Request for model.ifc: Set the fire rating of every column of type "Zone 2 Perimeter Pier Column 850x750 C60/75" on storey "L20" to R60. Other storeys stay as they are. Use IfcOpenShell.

First a look at what the model holds.

```python
import ifcopenshell
import ifcopenshell.util.element

model = ifcopenshell.open("model.ifc")
print(model.schema)
storey = next(s for s in model.by_type("IfcBuildingStorey") if s.Name == "L20")
columns = [e for e in ifcopenshell.util.element.get_decomposition(storey) if e.is_a("IfcColumn")]
seen = {}
for e in columns:
    element_type = ifcopenshell.util.element.get_type(e)
    key = (element_type.Name if element_type != e and element_type else None, ifcopenshell.util.element.get_pset(e, "Pset_ColumnCommon", "FireRating"))
    seen[key] = seen.get(key, 0) + 1
for (name, value), count in sorted(seen.items(), key=str):
    print(count, "x", name, "|", value)
```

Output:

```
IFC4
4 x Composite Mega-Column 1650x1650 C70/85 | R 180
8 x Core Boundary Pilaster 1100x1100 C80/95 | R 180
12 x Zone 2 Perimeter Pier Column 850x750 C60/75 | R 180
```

```python
import ifcopenshell
import ifcopenshell.api.pset
import ifcopenshell.util.element

model = ifcopenshell.open("model.ifc")

storey = next(s for s in model.by_type("IfcBuildingStorey") if s.Name == "L20")
columns = [e for e in ifcopenshell.util.element.get_decomposition(storey) if e.is_a("IfcColumn")]

count = 0
for e in columns:
    element_type = ifcopenshell.util.element.get_type(e)
    if element_type in (None, e) or element_type.Name != "Zone 2 Perimeter Pier Column 850x750 C60/75":
        continue
    found = ifcopenshell.util.element.get_pset(e, "Pset_ColumnCommon", should_inherit=False)
    if found:
        pset = model.by_id(found["id"])
        if len(ifcopenshell.util.element.get_elements_by_pset(pset)) > 1:
            pset = ifcopenshell.api.pset.unshare_pset(model, products=[e], pset=pset)[0]
    else:
        pset = ifcopenshell.api.pset.add_pset(model, product=e, name="Pset_ColumnCommon")
    ifcopenshell.api.pset.edit_pset(model, pset=pset, properties={"FireRating": "R60"})
    count += 1

print(count, "columns updated")

model.write("model_edited.ifc")
```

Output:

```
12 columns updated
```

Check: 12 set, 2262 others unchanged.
